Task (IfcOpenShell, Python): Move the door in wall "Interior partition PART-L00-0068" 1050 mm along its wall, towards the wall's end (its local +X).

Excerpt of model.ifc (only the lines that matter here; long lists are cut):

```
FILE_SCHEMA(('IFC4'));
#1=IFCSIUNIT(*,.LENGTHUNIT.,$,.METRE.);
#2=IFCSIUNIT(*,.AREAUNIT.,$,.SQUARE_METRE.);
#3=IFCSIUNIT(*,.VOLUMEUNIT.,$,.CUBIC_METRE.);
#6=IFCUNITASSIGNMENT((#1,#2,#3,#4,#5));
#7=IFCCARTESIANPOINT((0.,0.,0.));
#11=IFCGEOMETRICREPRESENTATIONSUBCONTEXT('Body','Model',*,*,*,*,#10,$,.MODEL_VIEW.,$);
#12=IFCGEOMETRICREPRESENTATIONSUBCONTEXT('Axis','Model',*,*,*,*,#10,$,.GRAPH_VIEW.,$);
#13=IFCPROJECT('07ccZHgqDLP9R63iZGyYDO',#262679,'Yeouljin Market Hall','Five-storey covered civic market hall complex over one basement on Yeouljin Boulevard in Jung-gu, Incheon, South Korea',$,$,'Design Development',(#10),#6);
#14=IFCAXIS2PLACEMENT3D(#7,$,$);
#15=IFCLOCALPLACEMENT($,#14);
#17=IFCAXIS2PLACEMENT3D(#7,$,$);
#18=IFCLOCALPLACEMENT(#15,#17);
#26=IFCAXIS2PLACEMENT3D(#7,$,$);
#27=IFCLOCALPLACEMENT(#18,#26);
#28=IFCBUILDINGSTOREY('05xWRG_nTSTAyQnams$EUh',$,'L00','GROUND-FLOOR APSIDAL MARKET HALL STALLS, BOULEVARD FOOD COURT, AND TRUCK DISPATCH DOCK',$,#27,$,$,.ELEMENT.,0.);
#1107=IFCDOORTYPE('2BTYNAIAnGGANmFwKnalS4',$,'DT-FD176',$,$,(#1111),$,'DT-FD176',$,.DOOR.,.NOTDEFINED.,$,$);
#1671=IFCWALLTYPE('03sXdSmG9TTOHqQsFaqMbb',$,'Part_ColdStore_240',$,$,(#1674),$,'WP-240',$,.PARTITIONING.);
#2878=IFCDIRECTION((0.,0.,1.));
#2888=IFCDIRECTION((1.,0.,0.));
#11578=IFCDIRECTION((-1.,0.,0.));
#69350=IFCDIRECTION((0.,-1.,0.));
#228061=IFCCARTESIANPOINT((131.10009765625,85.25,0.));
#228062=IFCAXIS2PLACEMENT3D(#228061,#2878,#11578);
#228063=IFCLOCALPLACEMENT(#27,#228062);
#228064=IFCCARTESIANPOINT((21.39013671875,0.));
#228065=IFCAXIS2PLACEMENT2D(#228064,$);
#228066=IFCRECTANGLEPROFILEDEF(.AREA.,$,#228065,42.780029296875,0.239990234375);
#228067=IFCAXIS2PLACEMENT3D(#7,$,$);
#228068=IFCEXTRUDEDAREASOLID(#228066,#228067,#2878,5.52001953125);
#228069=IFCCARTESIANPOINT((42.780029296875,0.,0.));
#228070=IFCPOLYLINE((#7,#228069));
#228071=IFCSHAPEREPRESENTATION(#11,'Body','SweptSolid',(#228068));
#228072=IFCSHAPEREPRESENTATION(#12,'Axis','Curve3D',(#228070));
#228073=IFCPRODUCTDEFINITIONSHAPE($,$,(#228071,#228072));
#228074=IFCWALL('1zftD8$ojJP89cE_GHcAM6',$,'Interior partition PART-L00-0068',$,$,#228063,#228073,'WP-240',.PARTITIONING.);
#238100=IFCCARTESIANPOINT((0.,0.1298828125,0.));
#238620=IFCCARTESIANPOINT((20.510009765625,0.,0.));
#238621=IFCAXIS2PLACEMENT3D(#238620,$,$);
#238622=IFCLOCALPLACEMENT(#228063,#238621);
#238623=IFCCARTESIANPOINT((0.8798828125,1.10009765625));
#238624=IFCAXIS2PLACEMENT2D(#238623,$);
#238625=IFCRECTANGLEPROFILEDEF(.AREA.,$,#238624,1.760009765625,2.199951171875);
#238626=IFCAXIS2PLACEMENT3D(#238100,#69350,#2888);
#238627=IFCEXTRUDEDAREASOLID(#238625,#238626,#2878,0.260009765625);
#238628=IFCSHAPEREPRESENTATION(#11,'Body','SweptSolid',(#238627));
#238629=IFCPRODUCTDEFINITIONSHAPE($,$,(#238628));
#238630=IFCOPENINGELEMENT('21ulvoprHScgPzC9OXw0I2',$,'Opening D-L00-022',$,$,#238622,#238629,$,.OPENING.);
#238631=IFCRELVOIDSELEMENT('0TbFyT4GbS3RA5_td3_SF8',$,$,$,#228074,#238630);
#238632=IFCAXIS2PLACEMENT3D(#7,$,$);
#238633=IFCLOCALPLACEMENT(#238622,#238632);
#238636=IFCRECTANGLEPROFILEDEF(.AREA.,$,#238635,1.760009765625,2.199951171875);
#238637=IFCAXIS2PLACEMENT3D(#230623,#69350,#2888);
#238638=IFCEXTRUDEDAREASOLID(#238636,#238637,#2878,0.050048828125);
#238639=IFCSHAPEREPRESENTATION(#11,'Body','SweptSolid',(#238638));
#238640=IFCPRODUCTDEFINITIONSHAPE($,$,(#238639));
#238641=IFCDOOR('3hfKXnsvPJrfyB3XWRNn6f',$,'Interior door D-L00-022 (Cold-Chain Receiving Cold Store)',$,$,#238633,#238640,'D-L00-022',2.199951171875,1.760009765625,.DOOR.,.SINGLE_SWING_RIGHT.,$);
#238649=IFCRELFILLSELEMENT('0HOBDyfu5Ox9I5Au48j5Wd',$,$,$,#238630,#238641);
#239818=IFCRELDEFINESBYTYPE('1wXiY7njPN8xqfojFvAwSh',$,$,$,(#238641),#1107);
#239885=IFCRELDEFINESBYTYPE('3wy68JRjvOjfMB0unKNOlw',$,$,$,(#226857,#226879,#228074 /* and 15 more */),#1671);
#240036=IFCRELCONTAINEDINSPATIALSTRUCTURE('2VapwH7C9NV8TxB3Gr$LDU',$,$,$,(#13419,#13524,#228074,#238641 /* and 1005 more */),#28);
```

```python
import ifcopenshell
import ifcopenshell.api.geometry
import ifcopenshell.util.placement
import ifcopenshell.util.unit

model = ifcopenshell.open("model.ifc")
unit_scale = ifcopenshell.util.unit.calculate_unit_scale(model)

door = model.by_id(238641)
opening = door.FillsVoids[0].RelatingOpeningElement
wall = opening.VoidsElements[0].RelatingBuildingElement

wall_matrix = ifcopenshell.util.placement.get_local_placement(wall.ObjectPlacement)
shift = wall_matrix[:3, 0] * 1.05 / unit_scale
before = ifcopenshell.util.placement.get_local_placement(door.ObjectPlacement)[:3, 3].copy()

# The door is placed relative to its opening, so it follows when the opening moves.
matrix = ifcopenshell.util.placement.get_local_placement(opening.ObjectPlacement)
matrix[:3, 3] += shift
ifcopenshell.api.geometry.edit_object_placement(
    model, product=opening, matrix=matrix, is_si=False, should_transform_children=True
)

after = ifcopenshell.util.placement.get_local_placement(door.ObjectPlacement)[:3, 3]
print("door moved by", (after - before).round(3) + 0.0)

model.write("model_updated.ifc")
```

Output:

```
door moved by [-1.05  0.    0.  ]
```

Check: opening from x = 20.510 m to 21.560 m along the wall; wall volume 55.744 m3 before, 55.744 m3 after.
